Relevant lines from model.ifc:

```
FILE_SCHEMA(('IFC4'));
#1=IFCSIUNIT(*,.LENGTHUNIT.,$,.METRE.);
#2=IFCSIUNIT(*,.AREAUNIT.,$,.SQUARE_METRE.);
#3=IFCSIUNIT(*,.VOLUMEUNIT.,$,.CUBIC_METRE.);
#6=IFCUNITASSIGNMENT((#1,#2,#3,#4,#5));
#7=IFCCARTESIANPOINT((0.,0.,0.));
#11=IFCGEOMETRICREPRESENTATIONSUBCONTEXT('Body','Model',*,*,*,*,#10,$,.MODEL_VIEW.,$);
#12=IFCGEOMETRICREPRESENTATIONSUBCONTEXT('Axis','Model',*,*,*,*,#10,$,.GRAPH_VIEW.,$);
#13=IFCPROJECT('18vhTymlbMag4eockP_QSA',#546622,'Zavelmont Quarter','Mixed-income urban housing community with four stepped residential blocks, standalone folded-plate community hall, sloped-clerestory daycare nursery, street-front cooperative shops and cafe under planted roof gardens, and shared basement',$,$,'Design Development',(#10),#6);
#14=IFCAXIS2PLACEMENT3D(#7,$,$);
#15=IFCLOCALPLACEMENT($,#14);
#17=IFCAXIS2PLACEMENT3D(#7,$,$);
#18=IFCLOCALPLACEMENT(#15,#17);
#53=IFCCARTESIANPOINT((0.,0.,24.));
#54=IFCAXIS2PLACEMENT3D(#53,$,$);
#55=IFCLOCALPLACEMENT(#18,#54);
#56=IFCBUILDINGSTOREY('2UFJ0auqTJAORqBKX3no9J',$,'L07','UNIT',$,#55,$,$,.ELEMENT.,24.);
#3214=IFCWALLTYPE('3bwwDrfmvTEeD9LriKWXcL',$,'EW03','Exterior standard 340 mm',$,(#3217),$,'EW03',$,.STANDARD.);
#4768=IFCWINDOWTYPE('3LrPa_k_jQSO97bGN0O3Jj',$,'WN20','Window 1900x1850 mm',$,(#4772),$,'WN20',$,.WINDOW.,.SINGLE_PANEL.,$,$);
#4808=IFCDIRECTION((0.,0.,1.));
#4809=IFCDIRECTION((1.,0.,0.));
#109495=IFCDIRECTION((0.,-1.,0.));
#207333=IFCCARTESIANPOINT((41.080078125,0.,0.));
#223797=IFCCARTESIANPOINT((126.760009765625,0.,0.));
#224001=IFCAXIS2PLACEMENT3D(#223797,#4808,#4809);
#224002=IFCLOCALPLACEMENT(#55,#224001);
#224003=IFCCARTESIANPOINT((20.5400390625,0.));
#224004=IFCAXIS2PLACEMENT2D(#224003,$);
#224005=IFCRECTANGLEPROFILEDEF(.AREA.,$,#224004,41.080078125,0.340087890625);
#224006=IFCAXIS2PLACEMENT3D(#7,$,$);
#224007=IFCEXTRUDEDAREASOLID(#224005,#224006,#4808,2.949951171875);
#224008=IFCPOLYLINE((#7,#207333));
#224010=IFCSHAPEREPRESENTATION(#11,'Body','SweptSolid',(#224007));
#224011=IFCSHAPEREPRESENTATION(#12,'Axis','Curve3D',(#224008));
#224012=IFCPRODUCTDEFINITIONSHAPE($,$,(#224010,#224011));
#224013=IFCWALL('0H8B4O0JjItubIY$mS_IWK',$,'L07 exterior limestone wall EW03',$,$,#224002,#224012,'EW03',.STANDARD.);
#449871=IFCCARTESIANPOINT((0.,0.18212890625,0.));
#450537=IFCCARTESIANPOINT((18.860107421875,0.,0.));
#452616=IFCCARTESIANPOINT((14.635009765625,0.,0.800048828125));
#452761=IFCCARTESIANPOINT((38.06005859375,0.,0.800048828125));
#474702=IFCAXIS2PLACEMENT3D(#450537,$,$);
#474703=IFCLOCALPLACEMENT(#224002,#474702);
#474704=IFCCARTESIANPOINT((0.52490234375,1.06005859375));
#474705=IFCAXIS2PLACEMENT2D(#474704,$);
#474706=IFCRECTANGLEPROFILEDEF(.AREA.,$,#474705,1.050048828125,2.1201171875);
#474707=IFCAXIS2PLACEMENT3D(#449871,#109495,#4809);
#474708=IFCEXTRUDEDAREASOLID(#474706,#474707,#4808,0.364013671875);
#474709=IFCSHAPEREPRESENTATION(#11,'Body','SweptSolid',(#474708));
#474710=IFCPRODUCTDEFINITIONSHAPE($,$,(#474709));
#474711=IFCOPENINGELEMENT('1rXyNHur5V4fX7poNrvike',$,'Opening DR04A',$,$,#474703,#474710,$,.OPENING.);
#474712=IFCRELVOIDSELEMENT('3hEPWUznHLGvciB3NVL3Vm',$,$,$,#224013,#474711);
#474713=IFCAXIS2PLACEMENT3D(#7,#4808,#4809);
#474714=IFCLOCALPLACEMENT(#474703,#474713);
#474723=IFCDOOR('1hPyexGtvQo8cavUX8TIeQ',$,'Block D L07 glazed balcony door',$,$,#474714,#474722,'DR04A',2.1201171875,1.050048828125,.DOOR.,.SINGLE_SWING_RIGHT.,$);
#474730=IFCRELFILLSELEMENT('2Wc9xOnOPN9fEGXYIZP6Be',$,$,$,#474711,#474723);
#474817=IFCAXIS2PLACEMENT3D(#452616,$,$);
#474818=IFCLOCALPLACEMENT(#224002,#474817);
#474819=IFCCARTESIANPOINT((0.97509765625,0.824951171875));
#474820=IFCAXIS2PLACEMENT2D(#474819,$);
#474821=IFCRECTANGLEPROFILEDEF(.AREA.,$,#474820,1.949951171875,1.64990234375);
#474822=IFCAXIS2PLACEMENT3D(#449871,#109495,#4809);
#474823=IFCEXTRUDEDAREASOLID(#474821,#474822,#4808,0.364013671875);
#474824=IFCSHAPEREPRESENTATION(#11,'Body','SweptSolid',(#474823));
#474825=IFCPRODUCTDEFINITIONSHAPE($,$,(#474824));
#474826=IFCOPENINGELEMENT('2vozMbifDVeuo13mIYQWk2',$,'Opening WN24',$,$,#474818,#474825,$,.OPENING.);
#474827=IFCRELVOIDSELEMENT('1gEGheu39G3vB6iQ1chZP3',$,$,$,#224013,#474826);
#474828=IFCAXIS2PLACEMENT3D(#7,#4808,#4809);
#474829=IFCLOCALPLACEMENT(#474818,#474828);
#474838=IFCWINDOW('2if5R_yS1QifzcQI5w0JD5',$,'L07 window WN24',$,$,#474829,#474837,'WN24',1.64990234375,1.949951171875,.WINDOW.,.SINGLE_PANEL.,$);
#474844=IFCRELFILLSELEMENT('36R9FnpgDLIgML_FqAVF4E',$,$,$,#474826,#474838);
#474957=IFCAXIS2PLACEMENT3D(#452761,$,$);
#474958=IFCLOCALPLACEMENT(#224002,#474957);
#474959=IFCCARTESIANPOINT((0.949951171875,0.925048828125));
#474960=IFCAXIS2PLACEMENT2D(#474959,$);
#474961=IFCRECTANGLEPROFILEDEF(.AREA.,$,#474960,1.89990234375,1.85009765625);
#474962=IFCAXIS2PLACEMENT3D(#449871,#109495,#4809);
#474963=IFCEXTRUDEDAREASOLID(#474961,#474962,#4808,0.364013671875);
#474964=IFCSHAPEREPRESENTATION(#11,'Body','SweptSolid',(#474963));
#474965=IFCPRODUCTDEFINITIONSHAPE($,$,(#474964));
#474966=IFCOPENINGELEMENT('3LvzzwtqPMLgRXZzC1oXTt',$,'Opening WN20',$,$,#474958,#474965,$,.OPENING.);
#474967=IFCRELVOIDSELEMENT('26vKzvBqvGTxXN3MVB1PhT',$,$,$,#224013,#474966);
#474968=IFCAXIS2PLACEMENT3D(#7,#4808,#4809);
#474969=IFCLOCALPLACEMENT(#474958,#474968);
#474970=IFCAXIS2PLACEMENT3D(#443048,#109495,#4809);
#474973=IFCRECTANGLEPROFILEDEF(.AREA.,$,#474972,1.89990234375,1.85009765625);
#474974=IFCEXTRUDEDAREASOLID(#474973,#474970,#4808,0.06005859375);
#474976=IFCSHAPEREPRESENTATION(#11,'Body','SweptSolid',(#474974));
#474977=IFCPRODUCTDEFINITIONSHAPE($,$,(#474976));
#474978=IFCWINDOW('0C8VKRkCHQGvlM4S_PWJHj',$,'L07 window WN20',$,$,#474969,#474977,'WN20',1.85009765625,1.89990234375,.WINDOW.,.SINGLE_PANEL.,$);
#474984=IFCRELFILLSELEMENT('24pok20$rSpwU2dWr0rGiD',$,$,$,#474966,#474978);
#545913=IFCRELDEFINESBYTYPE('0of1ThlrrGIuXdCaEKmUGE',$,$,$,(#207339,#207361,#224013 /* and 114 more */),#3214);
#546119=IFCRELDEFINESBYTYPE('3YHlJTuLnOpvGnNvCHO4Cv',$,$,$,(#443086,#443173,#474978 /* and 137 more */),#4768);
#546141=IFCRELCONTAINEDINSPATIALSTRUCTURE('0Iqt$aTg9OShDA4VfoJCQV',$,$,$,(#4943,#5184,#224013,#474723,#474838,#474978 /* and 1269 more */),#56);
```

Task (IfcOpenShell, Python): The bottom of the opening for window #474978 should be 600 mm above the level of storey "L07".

```python
import numpy as np
import ifcopenshell
import ifcopenshell.api.geometry
import ifcopenshell.geom
import ifcopenshell.util.element
import ifcopenshell.util.placement
import ifcopenshell.util.shape
import ifcopenshell.util.unit

model = ifcopenshell.open("model.ifc")
unit_scale = ifcopenshell.util.unit.calculate_unit_scale(model)

window = model.by_guid("0C8VKRkCHQGvlM4S_PWJHj")
opening = window.FillsVoids[0].RelatingOpeningElement
storey = ifcopenshell.util.element.get_container(window, ifc_class="IfcBuildingStorey")
level = ifcopenshell.util.placement.get_local_placement(storey.ObjectPlacement)[2, 3]

# The opening's origin need not be at the sill, so measure its lowest point.
shape = ifcopenshell.geom.create_shape(ifcopenshell.geom.settings(), opening)
bottom = ifcopenshell.util.shape.get_shape_bottom_elevation(shape, shape.geometry) / unit_scale
dz = level + 0.6 / unit_scale - bottom

shift = np.array([0.0, 0.0, dz])
# The window is placed relative to its opening, so it follows when the opening moves.
matrix = ifcopenshell.util.placement.get_local_placement(opening.ObjectPlacement)
matrix[:3, 3] += shift
ifcopenshell.api.geometry.edit_object_placement(
    model, product=opening, matrix=matrix, is_si=False, should_transform_children=True
)

print(f"moved by {dz * unit_scale:+.3f} m")

model.write("model_rev.ifc")
```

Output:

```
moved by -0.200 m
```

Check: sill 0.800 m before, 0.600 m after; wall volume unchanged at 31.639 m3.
